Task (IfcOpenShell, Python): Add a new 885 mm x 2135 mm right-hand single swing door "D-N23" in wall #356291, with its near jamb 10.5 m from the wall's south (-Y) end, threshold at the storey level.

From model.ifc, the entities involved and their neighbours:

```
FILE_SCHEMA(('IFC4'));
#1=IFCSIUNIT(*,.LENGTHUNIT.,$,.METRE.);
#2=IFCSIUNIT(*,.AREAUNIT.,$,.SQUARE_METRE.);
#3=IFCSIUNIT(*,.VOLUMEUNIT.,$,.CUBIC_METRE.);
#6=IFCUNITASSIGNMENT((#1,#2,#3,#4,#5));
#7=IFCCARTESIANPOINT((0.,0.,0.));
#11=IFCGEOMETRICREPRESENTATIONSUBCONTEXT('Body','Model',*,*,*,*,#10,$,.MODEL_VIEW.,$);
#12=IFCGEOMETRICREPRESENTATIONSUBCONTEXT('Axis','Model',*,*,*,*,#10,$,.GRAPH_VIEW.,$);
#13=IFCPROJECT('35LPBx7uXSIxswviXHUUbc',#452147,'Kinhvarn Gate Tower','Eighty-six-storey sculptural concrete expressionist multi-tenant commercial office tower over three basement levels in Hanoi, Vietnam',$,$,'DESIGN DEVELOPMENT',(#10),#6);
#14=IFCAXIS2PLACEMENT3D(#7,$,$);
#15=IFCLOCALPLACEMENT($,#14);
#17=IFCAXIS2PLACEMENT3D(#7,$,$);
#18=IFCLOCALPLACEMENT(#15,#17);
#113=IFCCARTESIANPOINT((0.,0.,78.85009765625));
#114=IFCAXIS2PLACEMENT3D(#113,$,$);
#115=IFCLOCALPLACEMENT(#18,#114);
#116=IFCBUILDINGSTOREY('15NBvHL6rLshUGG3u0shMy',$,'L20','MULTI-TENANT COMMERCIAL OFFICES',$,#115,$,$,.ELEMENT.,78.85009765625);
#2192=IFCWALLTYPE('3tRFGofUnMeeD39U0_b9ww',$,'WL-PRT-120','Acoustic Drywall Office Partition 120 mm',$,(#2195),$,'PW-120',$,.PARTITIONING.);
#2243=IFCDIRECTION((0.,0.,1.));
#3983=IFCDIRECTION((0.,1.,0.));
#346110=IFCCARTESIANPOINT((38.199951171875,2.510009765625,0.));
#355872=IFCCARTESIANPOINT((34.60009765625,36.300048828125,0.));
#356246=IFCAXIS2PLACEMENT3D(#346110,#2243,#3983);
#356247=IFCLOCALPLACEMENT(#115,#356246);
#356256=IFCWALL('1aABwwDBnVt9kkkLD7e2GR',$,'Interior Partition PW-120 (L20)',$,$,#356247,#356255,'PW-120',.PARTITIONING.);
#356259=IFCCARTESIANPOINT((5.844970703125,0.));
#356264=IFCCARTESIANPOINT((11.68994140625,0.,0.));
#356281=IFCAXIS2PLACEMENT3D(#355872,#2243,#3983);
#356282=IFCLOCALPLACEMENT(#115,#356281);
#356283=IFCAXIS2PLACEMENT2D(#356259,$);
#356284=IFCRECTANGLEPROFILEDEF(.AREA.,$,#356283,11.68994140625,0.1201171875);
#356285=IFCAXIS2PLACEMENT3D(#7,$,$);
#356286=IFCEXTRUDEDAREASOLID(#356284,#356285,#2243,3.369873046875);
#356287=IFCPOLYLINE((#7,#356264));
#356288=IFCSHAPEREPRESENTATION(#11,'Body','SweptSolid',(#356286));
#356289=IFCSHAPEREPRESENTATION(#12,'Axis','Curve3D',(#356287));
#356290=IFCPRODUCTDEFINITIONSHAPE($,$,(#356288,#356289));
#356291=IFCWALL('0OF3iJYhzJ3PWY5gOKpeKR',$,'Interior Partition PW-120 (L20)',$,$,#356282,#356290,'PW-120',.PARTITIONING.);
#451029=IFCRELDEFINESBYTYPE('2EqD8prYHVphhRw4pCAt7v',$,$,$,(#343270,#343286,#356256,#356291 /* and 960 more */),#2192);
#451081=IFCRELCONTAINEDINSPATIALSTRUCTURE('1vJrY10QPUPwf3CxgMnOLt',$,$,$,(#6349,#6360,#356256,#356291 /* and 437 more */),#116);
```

```python
import numpy as np
import ifcopenshell
import ifcopenshell.api.feature
import ifcopenshell.api.geometry
import ifcopenshell.api.root
import ifcopenshell.api.spatial
import ifcopenshell.geom
import ifcopenshell.util.element
import ifcopenshell.util.placement
import ifcopenshell.util.representation
import ifcopenshell.util.shape
import ifcopenshell.util.unit

model = ifcopenshell.open("model.ifc")
unit_scale = ifcopenshell.util.unit.calculate_unit_scale(model)
settings = ifcopenshell.geom.settings()


def volume(element):
    """Net volume in cubic metres, openings subtracted."""
    shape = ifcopenshell.geom.create_shape(settings, element)
    return ifcopenshell.util.shape.get_volume(shape.geometry)


wall = model.by_id(356291)
storey = ifcopenshell.util.element.get_container(wall, ifc_class="IfcBuildingStorey")
context = ifcopenshell.util.representation.get_context(model, "Model", "Body", "MODEL_VIEW")
before = volume(wall)

width, height, from_end, sill = 0.885, 2.135, 10.5, 0.0  # metres

# The wall runs along its own X axis, and the end named is its -X end.
wall_shape = ifcopenshell.geom.create_shape(settings, wall)
x, y, z = ifcopenshell.util.shape.get_vertices(wall_shape.geometry).T
start = x.min() + from_end
face, thickness = float(y.min()), float(y.max() - y.min())
wall_matrix = ifcopenshell.util.placement.get_local_placement(wall.ObjectPlacement)
level = ifcopenshell.util.placement.get_local_placement(storey.ObjectPlacement)[2, 3]


def in_wall(x, y):
    """Placement at x, y metres in the wall's axes, at sill height."""
    matrix = wall_matrix.copy()
    matrix[:, 3] = wall_matrix @ np.array([x / unit_scale, y / unit_scale, 0.0, 1.0])
    matrix[2, 3] = level + sill / unit_scale
    return matrix


# Opening: a box that overshoots both wall faces by 50 mm.
opening = ifcopenshell.api.root.create_entity(model, ifc_class="IfcOpeningElement", predefined_type="OPENING")
box = ifcopenshell.api.geometry.add_wall_representation(
    model, context=context, length=width, height=height, thickness=thickness + 0.1
)
ifcopenshell.api.geometry.assign_representation(model, product=opening, representation=box)
ifcopenshell.api.geometry.edit_object_placement(model, product=opening, matrix=in_wall(start, face - 0.05), is_si=False)
ifcopenshell.api.feature.add_feature(model, feature=opening, element=wall)

door = ifcopenshell.api.root.create_entity(model, ifc_class="IfcDoor", name="D-N23", predefined_type="DOOR")
door.OverallWidth, door.OverallHeight = width / unit_scale, height / unit_scale
door.OperationType = "SINGLE_SWING_RIGHT"
body = ifcopenshell.api.geometry.add_door_representation(
    model,
    context=context,
    overall_width=door.OverallWidth,
    overall_height=door.OverallHeight,
    operation_type="SINGLE_SWING_RIGHT",
    lining_properties={"LiningDepth": thickness / unit_scale, "ThresholdDepth": thickness / unit_scale},
)
ifcopenshell.api.geometry.assign_representation(model, product=door, representation=body)
ifcopenshell.api.spatial.assign_container(model, products=[door], relating_structure=storey)
ifcopenshell.api.feature.add_filling(model, opening=opening, element=door)

# The lining spans the wall, so the door starts at the wall face.
ifcopenshell.api.geometry.edit_object_placement(model, product=door, matrix=in_wall(start, face), is_si=False)

after = volume(wall)

print(f"wall volume {before:.3f} -> {after:.3f} m3")

model.write("model_edited.ifc")
```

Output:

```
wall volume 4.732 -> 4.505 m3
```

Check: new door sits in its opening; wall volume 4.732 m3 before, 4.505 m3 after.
